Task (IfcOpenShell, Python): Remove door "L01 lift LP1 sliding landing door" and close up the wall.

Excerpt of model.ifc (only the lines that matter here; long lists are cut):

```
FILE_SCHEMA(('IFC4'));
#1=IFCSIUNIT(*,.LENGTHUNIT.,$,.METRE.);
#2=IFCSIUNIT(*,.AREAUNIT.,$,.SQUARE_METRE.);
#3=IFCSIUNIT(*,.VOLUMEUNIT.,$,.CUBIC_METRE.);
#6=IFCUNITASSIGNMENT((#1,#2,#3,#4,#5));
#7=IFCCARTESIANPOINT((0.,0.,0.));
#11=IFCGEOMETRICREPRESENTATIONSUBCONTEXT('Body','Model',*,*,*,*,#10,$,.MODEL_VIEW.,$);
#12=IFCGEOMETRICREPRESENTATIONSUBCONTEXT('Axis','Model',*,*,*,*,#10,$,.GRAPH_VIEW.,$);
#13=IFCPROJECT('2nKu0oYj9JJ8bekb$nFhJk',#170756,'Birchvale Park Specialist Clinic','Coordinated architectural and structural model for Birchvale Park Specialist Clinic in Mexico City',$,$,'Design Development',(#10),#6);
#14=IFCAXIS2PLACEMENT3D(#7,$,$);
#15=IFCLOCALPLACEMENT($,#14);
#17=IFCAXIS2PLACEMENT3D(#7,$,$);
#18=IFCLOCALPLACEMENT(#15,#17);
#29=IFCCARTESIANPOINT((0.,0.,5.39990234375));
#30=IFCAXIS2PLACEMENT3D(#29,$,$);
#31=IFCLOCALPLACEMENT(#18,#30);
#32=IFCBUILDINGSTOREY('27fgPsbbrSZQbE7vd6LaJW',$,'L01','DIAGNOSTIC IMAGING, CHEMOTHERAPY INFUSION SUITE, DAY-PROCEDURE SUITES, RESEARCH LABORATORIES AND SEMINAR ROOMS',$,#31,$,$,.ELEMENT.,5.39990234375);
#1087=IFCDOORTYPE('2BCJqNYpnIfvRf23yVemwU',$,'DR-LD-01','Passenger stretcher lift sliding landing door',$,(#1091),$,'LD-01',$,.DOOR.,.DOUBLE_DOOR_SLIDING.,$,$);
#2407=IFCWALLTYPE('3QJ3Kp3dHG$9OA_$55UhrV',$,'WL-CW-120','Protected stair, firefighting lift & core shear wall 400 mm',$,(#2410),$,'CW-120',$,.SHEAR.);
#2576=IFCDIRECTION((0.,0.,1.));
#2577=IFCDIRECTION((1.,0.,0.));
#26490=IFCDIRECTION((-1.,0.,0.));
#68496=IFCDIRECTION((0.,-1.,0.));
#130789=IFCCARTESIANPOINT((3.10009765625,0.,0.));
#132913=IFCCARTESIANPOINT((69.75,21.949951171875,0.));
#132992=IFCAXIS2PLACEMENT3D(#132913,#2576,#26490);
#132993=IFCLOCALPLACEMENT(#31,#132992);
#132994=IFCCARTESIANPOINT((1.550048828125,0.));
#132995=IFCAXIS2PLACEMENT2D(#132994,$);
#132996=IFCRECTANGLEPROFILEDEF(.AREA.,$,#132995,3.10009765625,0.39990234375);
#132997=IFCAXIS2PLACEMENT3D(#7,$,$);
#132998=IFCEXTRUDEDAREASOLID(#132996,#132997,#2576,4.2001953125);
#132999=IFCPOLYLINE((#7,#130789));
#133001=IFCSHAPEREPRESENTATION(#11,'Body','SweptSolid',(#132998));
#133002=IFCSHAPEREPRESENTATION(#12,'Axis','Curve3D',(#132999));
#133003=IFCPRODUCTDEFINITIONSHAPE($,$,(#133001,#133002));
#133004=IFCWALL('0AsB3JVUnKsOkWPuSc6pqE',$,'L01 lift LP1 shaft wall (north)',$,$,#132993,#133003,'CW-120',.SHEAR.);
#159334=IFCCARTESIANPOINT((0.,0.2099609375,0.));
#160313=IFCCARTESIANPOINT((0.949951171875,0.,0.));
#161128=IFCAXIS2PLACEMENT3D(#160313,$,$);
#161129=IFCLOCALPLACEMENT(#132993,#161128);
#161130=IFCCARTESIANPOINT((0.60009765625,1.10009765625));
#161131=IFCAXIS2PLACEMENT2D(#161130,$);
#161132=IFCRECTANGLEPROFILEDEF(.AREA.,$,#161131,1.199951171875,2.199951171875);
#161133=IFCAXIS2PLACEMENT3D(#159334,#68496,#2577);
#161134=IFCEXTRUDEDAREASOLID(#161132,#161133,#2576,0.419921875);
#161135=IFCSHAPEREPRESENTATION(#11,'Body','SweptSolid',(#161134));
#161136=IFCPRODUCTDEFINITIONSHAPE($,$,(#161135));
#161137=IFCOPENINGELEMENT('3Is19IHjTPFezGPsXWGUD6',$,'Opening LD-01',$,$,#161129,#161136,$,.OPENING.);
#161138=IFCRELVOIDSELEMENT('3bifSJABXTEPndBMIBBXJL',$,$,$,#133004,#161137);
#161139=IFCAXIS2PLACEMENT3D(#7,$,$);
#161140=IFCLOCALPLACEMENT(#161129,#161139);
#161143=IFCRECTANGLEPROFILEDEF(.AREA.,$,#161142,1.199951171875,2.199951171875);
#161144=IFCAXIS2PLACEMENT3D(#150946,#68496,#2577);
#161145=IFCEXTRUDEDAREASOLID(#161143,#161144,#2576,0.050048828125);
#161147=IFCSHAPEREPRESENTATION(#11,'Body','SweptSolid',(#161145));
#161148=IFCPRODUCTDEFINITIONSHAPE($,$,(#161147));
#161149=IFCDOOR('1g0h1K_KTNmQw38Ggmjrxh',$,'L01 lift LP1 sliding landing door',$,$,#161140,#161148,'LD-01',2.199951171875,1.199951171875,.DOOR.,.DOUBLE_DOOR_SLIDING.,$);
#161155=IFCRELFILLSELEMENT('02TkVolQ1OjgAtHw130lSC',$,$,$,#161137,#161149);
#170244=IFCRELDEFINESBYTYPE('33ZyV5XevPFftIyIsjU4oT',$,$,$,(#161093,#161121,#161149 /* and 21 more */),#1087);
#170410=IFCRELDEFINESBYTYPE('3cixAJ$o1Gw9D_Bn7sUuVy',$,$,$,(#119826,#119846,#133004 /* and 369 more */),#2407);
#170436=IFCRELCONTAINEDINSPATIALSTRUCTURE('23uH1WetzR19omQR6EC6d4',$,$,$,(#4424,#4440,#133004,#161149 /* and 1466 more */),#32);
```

```python
import ifcopenshell
import ifcopenshell.api.feature
import ifcopenshell.api.root
import ifcopenshell.geom
import ifcopenshell.util.shape

model = ifcopenshell.open("model.ifc")
settings = ifcopenshell.geom.settings()


def volume(element):
    """Net volume in cubic metres, openings subtracted."""
    shape = ifcopenshell.geom.create_shape(settings, element)
    return ifcopenshell.util.shape.get_volume(shape.geometry)


door = model.by_guid("1g0h1K_KTNmQw38Ggmjrxh")
opening = door.FillsVoids[0].RelatingOpeningElement
wall = opening.VoidsElements[0].RelatingBuildingElement
before = volume(wall)

ifcopenshell.api.root.remove_product(model, product=door)
ifcopenshell.api.feature.remove_feature(model, feature=opening)

after = volume(wall)

print(f"wall volume {before:.3f} -> {after:.3f} m3")

model.write("model_updated.ifc")
```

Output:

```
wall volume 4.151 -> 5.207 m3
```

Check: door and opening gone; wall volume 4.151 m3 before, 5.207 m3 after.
